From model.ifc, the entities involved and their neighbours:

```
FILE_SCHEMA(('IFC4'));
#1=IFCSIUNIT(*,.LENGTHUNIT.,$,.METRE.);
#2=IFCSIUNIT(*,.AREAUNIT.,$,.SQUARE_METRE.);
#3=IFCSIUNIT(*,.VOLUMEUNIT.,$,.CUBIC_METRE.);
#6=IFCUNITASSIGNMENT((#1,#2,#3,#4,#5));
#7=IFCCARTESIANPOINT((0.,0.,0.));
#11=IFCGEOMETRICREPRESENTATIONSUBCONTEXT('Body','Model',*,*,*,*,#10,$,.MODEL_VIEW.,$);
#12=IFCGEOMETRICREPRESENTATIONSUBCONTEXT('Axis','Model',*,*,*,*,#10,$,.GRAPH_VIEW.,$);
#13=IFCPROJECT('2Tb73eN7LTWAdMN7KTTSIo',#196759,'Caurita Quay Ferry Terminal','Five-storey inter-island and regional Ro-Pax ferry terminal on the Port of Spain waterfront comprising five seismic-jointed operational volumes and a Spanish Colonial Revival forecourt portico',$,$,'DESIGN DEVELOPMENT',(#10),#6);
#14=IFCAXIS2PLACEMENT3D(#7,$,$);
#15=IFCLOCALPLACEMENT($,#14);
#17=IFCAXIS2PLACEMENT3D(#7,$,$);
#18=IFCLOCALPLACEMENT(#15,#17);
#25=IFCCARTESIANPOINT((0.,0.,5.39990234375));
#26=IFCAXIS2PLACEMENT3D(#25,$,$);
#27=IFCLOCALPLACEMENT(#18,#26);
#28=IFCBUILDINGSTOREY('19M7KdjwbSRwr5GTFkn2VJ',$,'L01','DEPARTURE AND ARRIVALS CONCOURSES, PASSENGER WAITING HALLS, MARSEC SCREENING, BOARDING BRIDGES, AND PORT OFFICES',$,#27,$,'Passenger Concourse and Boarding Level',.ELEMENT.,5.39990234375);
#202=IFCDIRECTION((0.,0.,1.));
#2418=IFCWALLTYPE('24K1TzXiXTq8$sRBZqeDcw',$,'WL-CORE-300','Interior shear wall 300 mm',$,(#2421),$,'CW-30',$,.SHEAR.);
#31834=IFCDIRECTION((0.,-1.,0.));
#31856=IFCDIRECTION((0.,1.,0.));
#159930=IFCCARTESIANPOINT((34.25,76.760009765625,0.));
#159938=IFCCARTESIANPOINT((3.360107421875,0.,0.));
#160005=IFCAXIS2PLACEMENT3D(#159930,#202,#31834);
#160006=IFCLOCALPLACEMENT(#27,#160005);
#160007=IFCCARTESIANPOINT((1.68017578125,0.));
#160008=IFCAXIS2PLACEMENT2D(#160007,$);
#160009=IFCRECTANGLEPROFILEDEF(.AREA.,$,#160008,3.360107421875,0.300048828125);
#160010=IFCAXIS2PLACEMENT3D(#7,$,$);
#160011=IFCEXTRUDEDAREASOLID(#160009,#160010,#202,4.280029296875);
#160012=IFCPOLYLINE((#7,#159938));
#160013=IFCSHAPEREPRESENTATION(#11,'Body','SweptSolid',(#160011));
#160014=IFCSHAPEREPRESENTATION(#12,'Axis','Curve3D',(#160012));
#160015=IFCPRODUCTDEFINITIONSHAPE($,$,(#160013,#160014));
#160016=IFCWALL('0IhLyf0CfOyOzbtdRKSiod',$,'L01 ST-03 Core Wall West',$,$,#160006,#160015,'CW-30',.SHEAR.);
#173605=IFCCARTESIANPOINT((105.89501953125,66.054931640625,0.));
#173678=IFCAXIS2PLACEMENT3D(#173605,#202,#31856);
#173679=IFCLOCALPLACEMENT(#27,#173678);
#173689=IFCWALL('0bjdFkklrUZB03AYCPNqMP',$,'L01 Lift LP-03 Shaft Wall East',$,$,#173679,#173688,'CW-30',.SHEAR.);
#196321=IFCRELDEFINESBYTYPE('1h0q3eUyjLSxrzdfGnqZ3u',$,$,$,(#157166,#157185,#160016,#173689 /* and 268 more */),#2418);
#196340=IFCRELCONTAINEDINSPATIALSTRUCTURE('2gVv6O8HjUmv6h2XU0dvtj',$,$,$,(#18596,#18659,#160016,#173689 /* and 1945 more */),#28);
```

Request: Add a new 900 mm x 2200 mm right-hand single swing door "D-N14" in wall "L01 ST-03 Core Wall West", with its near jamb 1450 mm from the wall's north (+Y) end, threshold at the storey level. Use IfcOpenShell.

```python
import numpy as np
import ifcopenshell
import ifcopenshell.api.feature
import ifcopenshell.api.geometry
import ifcopenshell.api.root
import ifcopenshell.api.spatial
import ifcopenshell.geom
import ifcopenshell.util.element
import ifcopenshell.util.placement
import ifcopenshell.util.representation
import ifcopenshell.util.shape
import ifcopenshell.util.unit

model = ifcopenshell.open("model.ifc")
unit_scale = ifcopenshell.util.unit.calculate_unit_scale(model)
settings = ifcopenshell.geom.settings()


def volume(element):
    """Net volume in cubic metres, openings subtracted."""
    shape = ifcopenshell.geom.create_shape(settings, element)
    return ifcopenshell.util.shape.get_volume(shape.geometry)


wall = model.by_guid("0IhLyf0CfOyOzbtdRKSiod")
storey = ifcopenshell.util.element.get_container(wall, ifc_class="IfcBuildingStorey")
context = ifcopenshell.util.representation.get_context(model, "Model", "Body", "MODEL_VIEW")
before = volume(wall)

width, height, from_end, sill = 0.9, 2.2, 1.45, 0.0  # metres

# The wall runs along its own X axis, and the end named is its -X end.
wall_shape = ifcopenshell.geom.create_shape(settings, wall)
x, y, z = ifcopenshell.util.shape.get_vertices(wall_shape.geometry).T
start = x.min() + from_end
face, thickness = float(y.min()), float(y.max() - y.min())
wall_matrix = ifcopenshell.util.placement.get_local_placement(wall.ObjectPlacement)
level = ifcopenshell.util.placement.get_local_placement(storey.ObjectPlacement)[2, 3]


def in_wall(x, y):
    """Placement at x, y metres in the wall's axes, at sill height."""
    matrix = wall_matrix.copy()
    matrix[:, 3] = wall_matrix @ np.array([x / unit_scale, y / unit_scale, 0.0, 1.0])
    matrix[2, 3] = level + sill / unit_scale
    return matrix


# Opening: a box that overshoots both wall faces by 50 mm.
opening = ifcopenshell.api.root.create_entity(model, ifc_class="IfcOpeningElement", predefined_type="OPENING")
box = ifcopenshell.api.geometry.add_wall_representation(
    model, context=context, length=width, height=height, thickness=thickness + 0.1
)
ifcopenshell.api.geometry.assign_representation(model, product=opening, representation=box)
ifcopenshell.api.geometry.edit_object_placement(model, product=opening, matrix=in_wall(start, face - 0.05), is_si=False)
ifcopenshell.api.feature.add_feature(model, feature=opening, element=wall)

door = ifcopenshell.api.root.create_entity(model, ifc_class="IfcDoor", name="D-N14", predefined_type="DOOR")
door.OverallWidth, door.OverallHeight = width / unit_scale, height / unit_scale
door.OperationType = "SINGLE_SWING_RIGHT"
body = ifcopenshell.api.geometry.add_door_representation(
    model,
    context=context,
    overall_width=door.OverallWidth,
    overall_height=door.OverallHeight,
    operation_type="SINGLE_SWING_RIGHT",
    lining_properties={"LiningDepth": thickness / unit_scale, "ThresholdDepth": thickness / unit_scale},
)
ifcopenshell.api.geometry.assign_representation(model, product=door, representation=body)
ifcopenshell.api.spatial.assign_container(model, products=[door], relating_structure=storey)
ifcopenshell.api.feature.add_filling(model, opening=opening, element=door)

# The lining spans the wall, so the door starts at the wall face.
ifcopenshell.api.geometry.edit_object_placement(model, product=door, matrix=in_wall(start, face), is_si=False)

after = volume(wall)

print(f"wall volume {before:.3f} -> {after:.3f} m3")

model.write("model-out.ifc")
```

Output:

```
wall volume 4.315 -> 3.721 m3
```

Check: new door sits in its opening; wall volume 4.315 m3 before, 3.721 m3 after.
